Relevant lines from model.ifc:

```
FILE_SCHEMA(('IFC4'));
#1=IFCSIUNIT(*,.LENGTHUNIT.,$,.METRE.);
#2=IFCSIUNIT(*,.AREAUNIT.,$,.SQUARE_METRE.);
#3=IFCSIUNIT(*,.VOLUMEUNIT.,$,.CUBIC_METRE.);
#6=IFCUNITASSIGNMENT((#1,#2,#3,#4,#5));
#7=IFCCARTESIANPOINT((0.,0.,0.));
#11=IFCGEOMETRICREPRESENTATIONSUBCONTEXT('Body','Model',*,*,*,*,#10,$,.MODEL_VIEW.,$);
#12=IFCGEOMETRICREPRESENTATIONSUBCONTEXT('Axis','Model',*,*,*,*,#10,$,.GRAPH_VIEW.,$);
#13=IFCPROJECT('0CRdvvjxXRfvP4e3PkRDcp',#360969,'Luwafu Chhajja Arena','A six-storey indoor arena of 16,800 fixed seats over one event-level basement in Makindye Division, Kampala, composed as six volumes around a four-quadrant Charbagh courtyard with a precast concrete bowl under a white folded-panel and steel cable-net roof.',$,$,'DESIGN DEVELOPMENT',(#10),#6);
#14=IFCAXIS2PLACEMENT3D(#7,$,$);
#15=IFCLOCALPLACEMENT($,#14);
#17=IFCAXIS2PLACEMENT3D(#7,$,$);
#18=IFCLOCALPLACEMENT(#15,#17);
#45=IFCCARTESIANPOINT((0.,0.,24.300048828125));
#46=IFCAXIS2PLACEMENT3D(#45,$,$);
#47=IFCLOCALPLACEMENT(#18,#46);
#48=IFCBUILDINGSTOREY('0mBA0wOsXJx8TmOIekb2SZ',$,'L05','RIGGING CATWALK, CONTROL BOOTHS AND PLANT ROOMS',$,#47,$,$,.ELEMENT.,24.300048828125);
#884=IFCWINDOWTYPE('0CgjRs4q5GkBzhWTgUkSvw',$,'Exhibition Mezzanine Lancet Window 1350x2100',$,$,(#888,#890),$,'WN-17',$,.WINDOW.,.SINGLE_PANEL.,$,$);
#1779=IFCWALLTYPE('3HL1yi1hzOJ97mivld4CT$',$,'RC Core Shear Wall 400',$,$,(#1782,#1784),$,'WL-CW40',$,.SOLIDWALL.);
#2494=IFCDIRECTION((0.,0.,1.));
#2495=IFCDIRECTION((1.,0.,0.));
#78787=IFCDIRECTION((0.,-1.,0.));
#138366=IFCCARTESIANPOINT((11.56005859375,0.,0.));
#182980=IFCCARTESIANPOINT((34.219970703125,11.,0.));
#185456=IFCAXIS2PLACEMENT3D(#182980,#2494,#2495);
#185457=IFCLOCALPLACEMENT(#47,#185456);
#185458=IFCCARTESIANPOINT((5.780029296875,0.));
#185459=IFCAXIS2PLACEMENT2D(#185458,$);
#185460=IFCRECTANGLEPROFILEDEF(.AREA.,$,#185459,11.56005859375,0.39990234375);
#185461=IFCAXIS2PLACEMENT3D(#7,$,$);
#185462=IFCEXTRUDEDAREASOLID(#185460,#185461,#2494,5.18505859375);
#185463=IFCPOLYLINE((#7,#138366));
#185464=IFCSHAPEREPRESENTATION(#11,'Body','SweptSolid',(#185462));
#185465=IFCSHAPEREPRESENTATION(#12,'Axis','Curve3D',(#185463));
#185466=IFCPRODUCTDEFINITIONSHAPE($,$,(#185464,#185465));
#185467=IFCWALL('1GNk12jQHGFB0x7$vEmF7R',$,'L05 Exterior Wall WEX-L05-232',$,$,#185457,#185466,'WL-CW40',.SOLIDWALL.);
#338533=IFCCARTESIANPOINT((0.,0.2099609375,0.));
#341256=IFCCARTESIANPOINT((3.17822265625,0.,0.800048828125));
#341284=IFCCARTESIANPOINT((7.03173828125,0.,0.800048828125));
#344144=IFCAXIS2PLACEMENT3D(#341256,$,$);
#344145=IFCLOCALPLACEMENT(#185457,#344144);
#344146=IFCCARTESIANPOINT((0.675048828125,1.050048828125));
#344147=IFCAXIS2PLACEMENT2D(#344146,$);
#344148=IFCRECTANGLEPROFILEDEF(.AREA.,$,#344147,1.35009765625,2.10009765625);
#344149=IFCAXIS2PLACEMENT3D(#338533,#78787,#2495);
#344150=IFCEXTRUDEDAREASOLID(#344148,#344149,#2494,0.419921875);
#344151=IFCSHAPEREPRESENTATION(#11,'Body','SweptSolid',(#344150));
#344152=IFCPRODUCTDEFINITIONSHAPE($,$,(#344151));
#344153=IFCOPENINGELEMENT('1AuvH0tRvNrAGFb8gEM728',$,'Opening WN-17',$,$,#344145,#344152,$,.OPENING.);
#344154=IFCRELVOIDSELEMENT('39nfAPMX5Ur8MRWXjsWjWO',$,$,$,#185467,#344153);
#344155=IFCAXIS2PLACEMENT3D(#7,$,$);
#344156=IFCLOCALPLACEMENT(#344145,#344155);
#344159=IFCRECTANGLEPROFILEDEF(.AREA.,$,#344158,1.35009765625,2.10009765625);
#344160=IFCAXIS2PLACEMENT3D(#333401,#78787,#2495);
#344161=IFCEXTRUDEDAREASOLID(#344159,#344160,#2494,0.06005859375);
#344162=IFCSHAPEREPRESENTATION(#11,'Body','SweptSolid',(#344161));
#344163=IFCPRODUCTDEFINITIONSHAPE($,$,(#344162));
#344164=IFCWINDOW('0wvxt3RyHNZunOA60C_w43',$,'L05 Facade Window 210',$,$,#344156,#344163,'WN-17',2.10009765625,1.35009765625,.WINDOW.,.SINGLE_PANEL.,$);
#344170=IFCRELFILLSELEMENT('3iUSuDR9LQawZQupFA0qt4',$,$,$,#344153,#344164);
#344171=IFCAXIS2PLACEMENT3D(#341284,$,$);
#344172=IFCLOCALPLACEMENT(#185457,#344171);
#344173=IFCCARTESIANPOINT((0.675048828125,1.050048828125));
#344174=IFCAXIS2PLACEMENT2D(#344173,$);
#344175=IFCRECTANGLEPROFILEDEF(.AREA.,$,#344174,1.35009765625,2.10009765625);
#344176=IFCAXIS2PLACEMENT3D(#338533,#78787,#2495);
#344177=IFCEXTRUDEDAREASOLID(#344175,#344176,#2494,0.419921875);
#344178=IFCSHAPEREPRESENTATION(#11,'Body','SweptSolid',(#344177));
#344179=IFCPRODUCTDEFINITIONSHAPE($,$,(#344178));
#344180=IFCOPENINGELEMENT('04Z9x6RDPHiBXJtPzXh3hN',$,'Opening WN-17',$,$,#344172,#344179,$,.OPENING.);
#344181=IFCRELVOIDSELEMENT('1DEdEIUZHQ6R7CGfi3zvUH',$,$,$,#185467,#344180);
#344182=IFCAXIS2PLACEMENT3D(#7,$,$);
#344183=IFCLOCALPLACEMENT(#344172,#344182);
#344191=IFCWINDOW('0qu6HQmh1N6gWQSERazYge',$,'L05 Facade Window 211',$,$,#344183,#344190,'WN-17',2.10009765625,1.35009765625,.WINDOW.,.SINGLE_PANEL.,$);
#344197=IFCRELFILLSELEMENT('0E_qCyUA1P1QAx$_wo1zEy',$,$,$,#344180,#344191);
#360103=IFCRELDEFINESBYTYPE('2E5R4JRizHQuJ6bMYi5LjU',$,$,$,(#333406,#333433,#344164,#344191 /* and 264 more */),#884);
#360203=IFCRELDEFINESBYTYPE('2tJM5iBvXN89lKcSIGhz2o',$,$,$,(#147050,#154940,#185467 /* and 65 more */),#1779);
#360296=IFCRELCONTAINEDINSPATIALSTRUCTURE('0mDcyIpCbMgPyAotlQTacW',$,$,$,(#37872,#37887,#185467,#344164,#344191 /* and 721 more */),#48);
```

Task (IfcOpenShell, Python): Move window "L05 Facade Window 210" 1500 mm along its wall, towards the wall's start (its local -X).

```python
import ifcopenshell
import ifcopenshell.api.geometry
import ifcopenshell.util.placement

model = ifcopenshell.open("model.ifc")

window = model.by_guid("0wvxt3RyHNZunOA60C_w43")
opening = window.FillsVoids[0].RelatingOpeningElement
wall = opening.VoidsElements[0].RelatingBuildingElement

wall_matrix = ifcopenshell.util.placement.get_local_placement(wall.ObjectPlacement)
shift = wall_matrix[:3, 0] * -1.5
before = ifcopenshell.util.placement.get_local_placement(window.ObjectPlacement)[:3, 3].copy()

# The window is placed relative to its opening, so it follows when the opening moves.
matrix = ifcopenshell.util.placement.get_local_placement(opening.ObjectPlacement)
matrix[:3, 3] += shift
ifcopenshell.api.geometry.edit_object_placement(
    model, product=opening, matrix=matrix, is_si=False, should_transform_children=True
)

after = ifcopenshell.util.placement.get_local_placement(window.ObjectPlacement)[:3, 3]
print("window moved by", (after - before).round(3) + 0.0)

model.write("model_rev.ifc")
```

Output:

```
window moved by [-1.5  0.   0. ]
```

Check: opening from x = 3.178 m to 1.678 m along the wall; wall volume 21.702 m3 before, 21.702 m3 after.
